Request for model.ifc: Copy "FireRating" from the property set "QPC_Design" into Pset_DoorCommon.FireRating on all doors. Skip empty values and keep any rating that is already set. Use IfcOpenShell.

First a look at what the model holds.

```python
import ifcopenshell
import ifcopenshell.util.element

model = ifcopenshell.open("model.ifc")
print(model.schema)
doors = model.by_type("IfcDoor")
print(len(doors), "doors")
for e in doors[:8]:
    source = ifcopenshell.util.element.get_pset(e, "QPC_Design", "FireRating")
    target = ifcopenshell.util.element.get_pset(e, "Pset_DoorCommon", "FireRating")
    print(e.id(), repr(source), repr(target), sep=" | ")
```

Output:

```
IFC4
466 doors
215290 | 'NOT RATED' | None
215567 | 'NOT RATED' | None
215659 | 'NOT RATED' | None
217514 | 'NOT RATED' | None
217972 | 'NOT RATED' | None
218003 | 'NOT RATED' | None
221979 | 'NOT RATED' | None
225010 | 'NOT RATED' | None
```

```python
import ifcopenshell
import ifcopenshell.api.pset
import ifcopenshell.util.element

model = ifcopenshell.open("model.ifc")

count = 0
for e in model.by_type("IfcDoor"):
    value = ifcopenshell.util.element.get_pset(e, "QPC_Design", "FireRating")
    current = ifcopenshell.util.element.get_pset(e, "Pset_DoorCommon", "FireRating")
    if not value or not value.strip() or current:
        continue
    # add_pset returns the element's existing set when there is one.
    pset = ifcopenshell.api.pset.add_pset(model, product=e, name="Pset_DoorCommon")
    ifcopenshell.api.pset.edit_pset(model, pset=pset, properties={"FireRating": value})
    count += 1

print(count, "doors updated")

model.write("model-out.ifc")
```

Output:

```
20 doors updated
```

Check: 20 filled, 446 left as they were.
